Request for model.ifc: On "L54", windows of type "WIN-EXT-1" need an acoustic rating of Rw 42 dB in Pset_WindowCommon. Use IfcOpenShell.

First a look at what the model holds.

```python
import ifcopenshell
import ifcopenshell.util.element

model = ifcopenshell.open("model.ifc")
print(model.schema)
storey = next(s for s in model.by_type("IfcBuildingStorey") if s.Name == "L54")
windows = [e for e in ifcopenshell.util.element.get_decomposition(storey) if e.is_a("IfcWindow")]
seen = {}
for e in windows:
    element_type = ifcopenshell.util.element.get_type(e)
    key = (element_type.Name if element_type != e and element_type else None, ifcopenshell.util.element.get_pset(e, "Pset_WindowCommon", "AcousticRating"))
    seen[key] = seen.get(key, 0) + 1
for (name, value), count in sorted(seen.items(), key=str):
    print(count, "x", name, "|", value)
```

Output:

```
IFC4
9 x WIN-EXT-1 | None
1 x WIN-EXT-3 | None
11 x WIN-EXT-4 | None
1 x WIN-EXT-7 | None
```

```python
import ifcopenshell
import ifcopenshell.api.pset
import ifcopenshell.util.element

model = ifcopenshell.open("model.ifc")

storey = next(s for s in model.by_type("IfcBuildingStorey") if s.Name == "L54")
windows = [e for e in ifcopenshell.util.element.get_decomposition(storey) if e.is_a("IfcWindow")]

count = 0
for e in windows:
    element_type = ifcopenshell.util.element.get_type(e)
    if element_type in (None, e) or element_type.Name != "WIN-EXT-1":
        continue
    found = ifcopenshell.util.element.get_pset(e, "Pset_WindowCommon", should_inherit=False)
    if found:
        pset = model.by_id(found["id"])
        if len(ifcopenshell.util.element.get_elements_by_pset(pset)) > 1:
            pset = ifcopenshell.api.pset.unshare_pset(model, products=[e], pset=pset)[0]
    else:
        pset = ifcopenshell.api.pset.add_pset(model, product=e, name="Pset_WindowCommon")
    ifcopenshell.api.pset.edit_pset(model, pset=pset, properties={"AcousticRating": "Rw 42 dB"})
    count += 1

print(count, "windows updated")

model.write("model-out.ifc")
```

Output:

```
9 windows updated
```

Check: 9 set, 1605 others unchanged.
